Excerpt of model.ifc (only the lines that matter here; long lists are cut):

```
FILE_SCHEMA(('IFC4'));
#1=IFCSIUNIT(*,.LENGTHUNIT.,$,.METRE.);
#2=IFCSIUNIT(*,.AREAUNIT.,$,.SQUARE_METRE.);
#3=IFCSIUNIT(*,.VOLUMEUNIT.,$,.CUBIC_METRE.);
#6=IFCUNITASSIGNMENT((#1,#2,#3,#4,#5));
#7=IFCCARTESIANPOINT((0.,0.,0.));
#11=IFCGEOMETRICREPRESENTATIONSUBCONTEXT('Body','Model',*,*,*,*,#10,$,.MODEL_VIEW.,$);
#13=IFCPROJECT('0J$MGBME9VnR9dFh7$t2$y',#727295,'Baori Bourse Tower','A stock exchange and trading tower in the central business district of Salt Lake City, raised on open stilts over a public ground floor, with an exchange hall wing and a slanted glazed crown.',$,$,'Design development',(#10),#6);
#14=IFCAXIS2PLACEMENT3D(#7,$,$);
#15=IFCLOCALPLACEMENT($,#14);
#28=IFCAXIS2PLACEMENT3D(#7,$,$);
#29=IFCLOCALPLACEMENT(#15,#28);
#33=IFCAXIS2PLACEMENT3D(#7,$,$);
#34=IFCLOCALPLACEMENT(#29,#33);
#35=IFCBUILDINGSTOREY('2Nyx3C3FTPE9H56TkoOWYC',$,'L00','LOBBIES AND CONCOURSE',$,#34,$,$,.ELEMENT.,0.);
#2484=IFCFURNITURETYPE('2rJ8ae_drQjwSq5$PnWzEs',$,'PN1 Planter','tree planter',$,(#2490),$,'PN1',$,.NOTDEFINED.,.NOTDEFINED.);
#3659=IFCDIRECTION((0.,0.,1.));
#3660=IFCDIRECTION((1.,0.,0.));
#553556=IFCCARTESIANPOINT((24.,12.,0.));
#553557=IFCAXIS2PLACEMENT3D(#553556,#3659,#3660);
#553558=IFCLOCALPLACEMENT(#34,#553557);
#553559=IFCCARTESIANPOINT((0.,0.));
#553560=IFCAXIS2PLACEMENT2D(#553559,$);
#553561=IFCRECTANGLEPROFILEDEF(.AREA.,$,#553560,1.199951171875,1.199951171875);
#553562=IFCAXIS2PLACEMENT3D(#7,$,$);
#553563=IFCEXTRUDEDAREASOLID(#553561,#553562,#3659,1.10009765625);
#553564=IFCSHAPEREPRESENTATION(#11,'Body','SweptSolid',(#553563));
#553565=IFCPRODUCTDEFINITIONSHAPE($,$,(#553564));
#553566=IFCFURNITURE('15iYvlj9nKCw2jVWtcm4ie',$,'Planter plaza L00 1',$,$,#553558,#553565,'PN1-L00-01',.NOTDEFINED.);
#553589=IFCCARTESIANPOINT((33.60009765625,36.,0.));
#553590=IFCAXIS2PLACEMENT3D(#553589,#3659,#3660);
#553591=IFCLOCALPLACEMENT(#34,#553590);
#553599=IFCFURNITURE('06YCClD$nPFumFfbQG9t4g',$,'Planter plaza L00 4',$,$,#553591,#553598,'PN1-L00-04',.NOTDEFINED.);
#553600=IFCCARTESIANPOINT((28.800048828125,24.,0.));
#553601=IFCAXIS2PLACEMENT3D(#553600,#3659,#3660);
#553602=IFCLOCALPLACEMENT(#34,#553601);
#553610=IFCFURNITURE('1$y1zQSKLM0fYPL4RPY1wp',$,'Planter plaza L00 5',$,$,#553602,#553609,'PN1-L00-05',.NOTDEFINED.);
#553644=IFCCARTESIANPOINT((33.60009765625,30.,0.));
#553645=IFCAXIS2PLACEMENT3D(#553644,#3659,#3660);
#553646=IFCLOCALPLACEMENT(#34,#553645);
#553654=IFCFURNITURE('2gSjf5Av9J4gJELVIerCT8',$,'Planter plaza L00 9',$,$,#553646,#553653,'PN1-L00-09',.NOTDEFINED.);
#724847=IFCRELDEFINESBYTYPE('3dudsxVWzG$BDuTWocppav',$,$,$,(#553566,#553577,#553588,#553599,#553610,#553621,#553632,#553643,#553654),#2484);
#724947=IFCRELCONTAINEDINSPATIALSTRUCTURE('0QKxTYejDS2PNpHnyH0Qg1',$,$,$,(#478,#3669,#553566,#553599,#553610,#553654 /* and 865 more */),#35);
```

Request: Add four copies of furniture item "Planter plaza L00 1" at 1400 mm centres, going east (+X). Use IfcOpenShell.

```python
import numpy as np
import ifcopenshell
import ifcopenshell.api.geometry
import ifcopenshell.api.root
import ifcopenshell.util.element
import ifcopenshell.util.placement
import ifcopenshell.util.unit

model = ifcopenshell.open("model.ifc")
unit_scale = ifcopenshell.util.unit.calculate_unit_scale(model)

source = model.by_guid("15iYvlj9nKCw2jVWtcm4ie")
base = ifcopenshell.util.placement.get_local_placement(source.ObjectPlacement)
step = np.array([1.0, 0.0, 0.0]) * 1.4 / unit_scale

for i in range(1, 5):
    copy = ifcopenshell.api.root.copy_class(model, product=source)
    copy.Representation = ifcopenshell.util.element.copy_deep(
        model, source.Representation, exclude=["IfcGeometricRepresentationContext", "IfcRepresentationMap"]
    )
    copy.Tag = None
    matrix = base.copy()
    matrix[:3, 3] += i * step
    print("added at", matrix[:3, 3].round(3) + 0.0)
    ifcopenshell.api.geometry.edit_object_placement(model, product=copy, matrix=matrix, is_si=False)

model.write("model-out.ifc")
```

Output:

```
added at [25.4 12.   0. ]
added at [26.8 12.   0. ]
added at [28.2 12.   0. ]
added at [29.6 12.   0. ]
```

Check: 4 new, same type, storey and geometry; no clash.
